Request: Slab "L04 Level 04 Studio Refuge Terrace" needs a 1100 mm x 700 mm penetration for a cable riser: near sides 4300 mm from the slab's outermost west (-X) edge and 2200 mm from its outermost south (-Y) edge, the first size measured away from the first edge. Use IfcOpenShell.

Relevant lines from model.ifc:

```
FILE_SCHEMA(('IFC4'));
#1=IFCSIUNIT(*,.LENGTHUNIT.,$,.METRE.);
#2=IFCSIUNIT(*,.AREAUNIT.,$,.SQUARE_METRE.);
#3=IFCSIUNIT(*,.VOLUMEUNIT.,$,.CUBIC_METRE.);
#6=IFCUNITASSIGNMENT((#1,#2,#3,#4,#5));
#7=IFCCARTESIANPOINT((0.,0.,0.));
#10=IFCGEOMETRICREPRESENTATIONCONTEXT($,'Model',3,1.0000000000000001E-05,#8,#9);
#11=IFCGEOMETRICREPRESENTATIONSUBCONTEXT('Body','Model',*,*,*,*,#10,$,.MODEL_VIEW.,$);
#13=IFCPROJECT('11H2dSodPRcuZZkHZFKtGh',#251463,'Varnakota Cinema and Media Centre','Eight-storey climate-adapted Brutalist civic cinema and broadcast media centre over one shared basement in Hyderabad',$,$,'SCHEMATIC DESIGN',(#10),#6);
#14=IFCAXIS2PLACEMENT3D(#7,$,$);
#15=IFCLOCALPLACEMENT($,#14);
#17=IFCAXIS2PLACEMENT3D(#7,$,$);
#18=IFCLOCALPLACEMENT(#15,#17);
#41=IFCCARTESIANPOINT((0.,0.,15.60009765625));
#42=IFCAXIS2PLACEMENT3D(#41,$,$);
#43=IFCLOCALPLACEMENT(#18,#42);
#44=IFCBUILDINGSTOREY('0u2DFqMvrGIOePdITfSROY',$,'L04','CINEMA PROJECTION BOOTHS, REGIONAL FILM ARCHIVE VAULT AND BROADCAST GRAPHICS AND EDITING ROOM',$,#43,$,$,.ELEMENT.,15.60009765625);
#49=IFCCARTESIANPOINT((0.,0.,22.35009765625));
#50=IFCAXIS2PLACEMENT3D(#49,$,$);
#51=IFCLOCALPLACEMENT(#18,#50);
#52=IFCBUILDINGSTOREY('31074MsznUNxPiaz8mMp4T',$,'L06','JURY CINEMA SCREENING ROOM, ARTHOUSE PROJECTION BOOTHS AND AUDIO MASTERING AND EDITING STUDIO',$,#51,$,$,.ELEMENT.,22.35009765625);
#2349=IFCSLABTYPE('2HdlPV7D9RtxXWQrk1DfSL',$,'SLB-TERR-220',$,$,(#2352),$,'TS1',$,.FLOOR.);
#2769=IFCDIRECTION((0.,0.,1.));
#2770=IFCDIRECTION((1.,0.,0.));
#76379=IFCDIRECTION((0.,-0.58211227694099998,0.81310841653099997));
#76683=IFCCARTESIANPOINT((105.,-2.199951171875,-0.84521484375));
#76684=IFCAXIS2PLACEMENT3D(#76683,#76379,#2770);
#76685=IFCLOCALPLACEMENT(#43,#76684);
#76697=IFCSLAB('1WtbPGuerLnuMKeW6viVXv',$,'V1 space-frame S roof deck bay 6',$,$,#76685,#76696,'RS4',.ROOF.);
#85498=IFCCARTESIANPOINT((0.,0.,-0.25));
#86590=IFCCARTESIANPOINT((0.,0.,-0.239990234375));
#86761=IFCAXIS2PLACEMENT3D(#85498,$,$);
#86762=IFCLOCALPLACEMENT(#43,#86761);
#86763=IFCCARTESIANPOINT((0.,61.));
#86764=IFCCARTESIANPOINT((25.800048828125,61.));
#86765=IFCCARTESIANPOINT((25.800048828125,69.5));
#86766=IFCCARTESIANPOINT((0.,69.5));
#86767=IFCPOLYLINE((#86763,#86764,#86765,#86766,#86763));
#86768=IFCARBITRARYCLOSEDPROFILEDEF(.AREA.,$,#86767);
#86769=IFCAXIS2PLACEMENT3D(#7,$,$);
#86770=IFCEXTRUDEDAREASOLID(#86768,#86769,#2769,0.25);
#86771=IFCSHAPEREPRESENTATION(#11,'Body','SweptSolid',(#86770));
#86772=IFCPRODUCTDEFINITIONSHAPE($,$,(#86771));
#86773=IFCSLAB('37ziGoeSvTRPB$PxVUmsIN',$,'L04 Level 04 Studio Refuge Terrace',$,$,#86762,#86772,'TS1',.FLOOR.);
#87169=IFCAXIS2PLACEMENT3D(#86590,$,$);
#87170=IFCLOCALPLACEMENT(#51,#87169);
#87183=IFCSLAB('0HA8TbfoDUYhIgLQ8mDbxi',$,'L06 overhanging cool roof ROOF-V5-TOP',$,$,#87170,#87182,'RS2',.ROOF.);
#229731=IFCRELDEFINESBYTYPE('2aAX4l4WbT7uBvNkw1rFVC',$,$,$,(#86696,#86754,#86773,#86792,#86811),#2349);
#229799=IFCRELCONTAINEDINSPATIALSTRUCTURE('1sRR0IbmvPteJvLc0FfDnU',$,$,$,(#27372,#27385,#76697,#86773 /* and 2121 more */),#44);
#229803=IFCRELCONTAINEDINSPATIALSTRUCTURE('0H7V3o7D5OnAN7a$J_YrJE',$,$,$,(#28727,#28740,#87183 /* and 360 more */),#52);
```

```python
import numpy as np
import ifcopenshell
import ifcopenshell.api.feature
import ifcopenshell.api.geometry
import ifcopenshell.api.root
import ifcopenshell.geom
import ifcopenshell.util.placement
import ifcopenshell.util.representation
import ifcopenshell.util.shape
import ifcopenshell.util.unit

model = ifcopenshell.open("model.ifc")
unit_scale = ifcopenshell.util.unit.calculate_unit_scale(model)
settings = ifcopenshell.geom.settings()


def volume(element):
    """Net volume in cubic metres, openings subtracted."""
    shape = ifcopenshell.geom.create_shape(settings, element)
    return ifcopenshell.util.shape.get_volume(shape.geometry)


slab = model.by_guid("37ziGoeSvTRPB$PxVUmsIN")
before = volume(slab)

# Extent in the slab's own axes, in metres. The edges named are its -X and -Y sides.
slab_shape = ifcopenshell.geom.create_shape(settings, slab)
vertices = ifcopenshell.util.shape.get_vertices(slab_shape.geometry)
x_min, y_min, bottom = vertices.min(axis=0)
top = vertices[:, 2].max()

opening = ifcopenshell.api.root.create_entity(model, ifc_class="IfcOpeningElement", name="Cable riser opening", predefined_type="OPENING")
context = ifcopenshell.util.representation.get_context(model, "Model", "Body", "MODEL_VIEW")
width, depth = 1.1, 0.7
outline = [(0.0, 0.0), (width, 0.0), (width, depth), (0.0, depth), (0.0, 0.0)]
# Overshoot both faces by 50 mm so the cut is clean.
shape = ifcopenshell.api.geometry.add_slab_representation(
    model, context=context, depth=top - bottom + 0.1, polyline=outline
)
ifcopenshell.api.geometry.assign_representation(model, product=opening, representation=shape)

matrix = ifcopenshell.util.placement.get_local_placement(slab.ObjectPlacement)
matrix[:, 3] = matrix @ np.append(np.array([x_min + 4.3, y_min + 2.2, bottom - 0.05]) / unit_scale, 1.0)
ifcopenshell.api.geometry.edit_object_placement(model, product=opening, matrix=matrix, is_si=False)
ifcopenshell.api.feature.add_feature(model, feature=opening, element=slab)

after = volume(slab)

print(f"slab volume {before:.3f} -> {after:.3f} m3")

model.write("model_edited.ifc")
```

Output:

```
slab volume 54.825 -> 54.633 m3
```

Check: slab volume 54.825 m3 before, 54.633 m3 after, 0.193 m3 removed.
